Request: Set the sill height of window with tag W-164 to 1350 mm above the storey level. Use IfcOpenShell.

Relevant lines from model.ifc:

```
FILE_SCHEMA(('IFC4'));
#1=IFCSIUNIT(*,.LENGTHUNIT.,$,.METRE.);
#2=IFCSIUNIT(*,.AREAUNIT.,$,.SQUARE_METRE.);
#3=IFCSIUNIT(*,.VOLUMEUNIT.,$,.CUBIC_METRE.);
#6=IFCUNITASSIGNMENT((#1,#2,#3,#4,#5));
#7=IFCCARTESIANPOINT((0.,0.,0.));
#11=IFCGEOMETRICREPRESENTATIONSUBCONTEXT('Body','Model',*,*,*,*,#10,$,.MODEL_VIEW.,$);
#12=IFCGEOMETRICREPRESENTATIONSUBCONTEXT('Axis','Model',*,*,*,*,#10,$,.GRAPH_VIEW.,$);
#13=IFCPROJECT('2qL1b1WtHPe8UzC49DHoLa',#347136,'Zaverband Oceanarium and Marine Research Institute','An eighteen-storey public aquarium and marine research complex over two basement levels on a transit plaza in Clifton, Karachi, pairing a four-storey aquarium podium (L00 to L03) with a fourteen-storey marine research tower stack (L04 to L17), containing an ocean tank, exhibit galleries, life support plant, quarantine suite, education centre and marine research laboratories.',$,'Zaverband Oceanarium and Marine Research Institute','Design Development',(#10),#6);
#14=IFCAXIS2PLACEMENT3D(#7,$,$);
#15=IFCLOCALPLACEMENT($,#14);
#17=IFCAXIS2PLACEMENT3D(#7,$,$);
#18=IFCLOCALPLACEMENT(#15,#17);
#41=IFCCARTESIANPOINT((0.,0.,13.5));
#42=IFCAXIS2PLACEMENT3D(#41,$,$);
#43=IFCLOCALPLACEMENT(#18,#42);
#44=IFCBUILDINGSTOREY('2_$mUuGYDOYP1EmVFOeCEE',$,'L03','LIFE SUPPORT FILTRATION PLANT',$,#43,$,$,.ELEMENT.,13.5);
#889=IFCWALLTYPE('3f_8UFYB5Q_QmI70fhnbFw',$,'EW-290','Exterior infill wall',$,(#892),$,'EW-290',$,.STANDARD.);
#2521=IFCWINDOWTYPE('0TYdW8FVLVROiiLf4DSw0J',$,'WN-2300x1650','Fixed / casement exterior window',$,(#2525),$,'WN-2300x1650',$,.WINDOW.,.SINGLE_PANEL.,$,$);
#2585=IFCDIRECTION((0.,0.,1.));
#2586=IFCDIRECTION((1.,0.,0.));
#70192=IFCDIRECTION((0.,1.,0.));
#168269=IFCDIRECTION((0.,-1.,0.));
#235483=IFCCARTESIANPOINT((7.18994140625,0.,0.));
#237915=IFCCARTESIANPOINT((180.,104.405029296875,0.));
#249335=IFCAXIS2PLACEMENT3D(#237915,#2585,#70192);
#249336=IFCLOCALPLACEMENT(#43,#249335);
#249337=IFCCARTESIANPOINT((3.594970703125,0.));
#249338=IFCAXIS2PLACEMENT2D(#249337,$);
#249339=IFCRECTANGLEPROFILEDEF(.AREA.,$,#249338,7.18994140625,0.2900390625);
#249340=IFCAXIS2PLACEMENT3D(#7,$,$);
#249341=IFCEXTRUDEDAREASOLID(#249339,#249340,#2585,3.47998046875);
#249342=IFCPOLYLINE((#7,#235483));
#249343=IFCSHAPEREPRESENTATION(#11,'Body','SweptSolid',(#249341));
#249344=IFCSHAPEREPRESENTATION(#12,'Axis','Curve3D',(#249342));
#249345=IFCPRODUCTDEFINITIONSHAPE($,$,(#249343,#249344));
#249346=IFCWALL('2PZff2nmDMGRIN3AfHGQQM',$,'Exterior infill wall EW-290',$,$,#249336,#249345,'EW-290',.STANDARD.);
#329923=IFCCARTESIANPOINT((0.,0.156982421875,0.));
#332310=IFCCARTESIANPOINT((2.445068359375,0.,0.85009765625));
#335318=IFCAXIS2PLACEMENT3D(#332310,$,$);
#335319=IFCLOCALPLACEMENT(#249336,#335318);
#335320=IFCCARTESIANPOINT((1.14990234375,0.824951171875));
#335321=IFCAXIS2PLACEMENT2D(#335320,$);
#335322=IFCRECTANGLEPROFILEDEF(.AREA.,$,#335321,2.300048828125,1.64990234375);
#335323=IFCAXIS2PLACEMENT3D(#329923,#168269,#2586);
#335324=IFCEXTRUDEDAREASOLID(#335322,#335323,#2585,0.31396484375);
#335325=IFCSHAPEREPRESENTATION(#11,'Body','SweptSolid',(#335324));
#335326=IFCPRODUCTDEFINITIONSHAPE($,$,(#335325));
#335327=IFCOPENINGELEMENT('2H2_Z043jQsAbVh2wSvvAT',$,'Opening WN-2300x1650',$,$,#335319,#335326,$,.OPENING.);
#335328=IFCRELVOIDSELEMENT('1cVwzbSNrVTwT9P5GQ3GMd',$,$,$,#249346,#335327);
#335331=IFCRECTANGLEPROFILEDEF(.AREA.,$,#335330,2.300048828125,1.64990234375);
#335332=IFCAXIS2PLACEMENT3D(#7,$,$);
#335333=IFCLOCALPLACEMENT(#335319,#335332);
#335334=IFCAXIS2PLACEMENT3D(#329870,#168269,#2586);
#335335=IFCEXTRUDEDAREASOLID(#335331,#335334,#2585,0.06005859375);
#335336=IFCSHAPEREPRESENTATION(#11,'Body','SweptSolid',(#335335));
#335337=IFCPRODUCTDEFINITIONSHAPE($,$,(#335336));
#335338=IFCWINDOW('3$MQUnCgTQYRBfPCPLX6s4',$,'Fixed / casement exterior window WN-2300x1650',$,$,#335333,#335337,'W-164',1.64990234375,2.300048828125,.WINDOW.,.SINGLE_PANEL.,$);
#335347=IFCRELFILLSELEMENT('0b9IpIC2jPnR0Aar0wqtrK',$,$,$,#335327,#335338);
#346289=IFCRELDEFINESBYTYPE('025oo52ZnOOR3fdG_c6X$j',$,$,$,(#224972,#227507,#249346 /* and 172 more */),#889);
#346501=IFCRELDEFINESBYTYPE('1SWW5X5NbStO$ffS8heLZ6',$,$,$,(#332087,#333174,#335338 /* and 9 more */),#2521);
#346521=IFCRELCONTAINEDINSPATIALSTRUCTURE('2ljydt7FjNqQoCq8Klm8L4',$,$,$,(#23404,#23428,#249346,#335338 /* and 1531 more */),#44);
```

```python
import numpy as np
import ifcopenshell
import ifcopenshell.api.geometry
import ifcopenshell.geom
import ifcopenshell.util.element
import ifcopenshell.util.placement
import ifcopenshell.util.shape
import ifcopenshell.util.unit

model = ifcopenshell.open("model.ifc")
unit_scale = ifcopenshell.util.unit.calculate_unit_scale(model)

window = model.by_guid("3$MQUnCgTQYRBfPCPLX6s4")
opening = window.FillsVoids[0].RelatingOpeningElement
storey = ifcopenshell.util.element.get_container(window, ifc_class="IfcBuildingStorey")
level = ifcopenshell.util.placement.get_local_placement(storey.ObjectPlacement)[2, 3]

# The opening's origin need not be at the sill, so measure its lowest point.
shape = ifcopenshell.geom.create_shape(ifcopenshell.geom.settings(), opening)
bottom = ifcopenshell.util.shape.get_shape_bottom_elevation(shape, shape.geometry) / unit_scale
dz = level + 1.35 / unit_scale - bottom

shift = np.array([0.0, 0.0, dz])
# The window is placed relative to its opening, so it follows when the opening moves.
matrix = ifcopenshell.util.placement.get_local_placement(opening.ObjectPlacement)
matrix[:3, 3] += shift
ifcopenshell.api.geometry.edit_object_placement(
    model, product=opening, matrix=matrix, is_si=False, should_transform_children=True
)

print(f"moved by {dz * unit_scale:+.3f} m")

model.write("model_rev.ifc")
```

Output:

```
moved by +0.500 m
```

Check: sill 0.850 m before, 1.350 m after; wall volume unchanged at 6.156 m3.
